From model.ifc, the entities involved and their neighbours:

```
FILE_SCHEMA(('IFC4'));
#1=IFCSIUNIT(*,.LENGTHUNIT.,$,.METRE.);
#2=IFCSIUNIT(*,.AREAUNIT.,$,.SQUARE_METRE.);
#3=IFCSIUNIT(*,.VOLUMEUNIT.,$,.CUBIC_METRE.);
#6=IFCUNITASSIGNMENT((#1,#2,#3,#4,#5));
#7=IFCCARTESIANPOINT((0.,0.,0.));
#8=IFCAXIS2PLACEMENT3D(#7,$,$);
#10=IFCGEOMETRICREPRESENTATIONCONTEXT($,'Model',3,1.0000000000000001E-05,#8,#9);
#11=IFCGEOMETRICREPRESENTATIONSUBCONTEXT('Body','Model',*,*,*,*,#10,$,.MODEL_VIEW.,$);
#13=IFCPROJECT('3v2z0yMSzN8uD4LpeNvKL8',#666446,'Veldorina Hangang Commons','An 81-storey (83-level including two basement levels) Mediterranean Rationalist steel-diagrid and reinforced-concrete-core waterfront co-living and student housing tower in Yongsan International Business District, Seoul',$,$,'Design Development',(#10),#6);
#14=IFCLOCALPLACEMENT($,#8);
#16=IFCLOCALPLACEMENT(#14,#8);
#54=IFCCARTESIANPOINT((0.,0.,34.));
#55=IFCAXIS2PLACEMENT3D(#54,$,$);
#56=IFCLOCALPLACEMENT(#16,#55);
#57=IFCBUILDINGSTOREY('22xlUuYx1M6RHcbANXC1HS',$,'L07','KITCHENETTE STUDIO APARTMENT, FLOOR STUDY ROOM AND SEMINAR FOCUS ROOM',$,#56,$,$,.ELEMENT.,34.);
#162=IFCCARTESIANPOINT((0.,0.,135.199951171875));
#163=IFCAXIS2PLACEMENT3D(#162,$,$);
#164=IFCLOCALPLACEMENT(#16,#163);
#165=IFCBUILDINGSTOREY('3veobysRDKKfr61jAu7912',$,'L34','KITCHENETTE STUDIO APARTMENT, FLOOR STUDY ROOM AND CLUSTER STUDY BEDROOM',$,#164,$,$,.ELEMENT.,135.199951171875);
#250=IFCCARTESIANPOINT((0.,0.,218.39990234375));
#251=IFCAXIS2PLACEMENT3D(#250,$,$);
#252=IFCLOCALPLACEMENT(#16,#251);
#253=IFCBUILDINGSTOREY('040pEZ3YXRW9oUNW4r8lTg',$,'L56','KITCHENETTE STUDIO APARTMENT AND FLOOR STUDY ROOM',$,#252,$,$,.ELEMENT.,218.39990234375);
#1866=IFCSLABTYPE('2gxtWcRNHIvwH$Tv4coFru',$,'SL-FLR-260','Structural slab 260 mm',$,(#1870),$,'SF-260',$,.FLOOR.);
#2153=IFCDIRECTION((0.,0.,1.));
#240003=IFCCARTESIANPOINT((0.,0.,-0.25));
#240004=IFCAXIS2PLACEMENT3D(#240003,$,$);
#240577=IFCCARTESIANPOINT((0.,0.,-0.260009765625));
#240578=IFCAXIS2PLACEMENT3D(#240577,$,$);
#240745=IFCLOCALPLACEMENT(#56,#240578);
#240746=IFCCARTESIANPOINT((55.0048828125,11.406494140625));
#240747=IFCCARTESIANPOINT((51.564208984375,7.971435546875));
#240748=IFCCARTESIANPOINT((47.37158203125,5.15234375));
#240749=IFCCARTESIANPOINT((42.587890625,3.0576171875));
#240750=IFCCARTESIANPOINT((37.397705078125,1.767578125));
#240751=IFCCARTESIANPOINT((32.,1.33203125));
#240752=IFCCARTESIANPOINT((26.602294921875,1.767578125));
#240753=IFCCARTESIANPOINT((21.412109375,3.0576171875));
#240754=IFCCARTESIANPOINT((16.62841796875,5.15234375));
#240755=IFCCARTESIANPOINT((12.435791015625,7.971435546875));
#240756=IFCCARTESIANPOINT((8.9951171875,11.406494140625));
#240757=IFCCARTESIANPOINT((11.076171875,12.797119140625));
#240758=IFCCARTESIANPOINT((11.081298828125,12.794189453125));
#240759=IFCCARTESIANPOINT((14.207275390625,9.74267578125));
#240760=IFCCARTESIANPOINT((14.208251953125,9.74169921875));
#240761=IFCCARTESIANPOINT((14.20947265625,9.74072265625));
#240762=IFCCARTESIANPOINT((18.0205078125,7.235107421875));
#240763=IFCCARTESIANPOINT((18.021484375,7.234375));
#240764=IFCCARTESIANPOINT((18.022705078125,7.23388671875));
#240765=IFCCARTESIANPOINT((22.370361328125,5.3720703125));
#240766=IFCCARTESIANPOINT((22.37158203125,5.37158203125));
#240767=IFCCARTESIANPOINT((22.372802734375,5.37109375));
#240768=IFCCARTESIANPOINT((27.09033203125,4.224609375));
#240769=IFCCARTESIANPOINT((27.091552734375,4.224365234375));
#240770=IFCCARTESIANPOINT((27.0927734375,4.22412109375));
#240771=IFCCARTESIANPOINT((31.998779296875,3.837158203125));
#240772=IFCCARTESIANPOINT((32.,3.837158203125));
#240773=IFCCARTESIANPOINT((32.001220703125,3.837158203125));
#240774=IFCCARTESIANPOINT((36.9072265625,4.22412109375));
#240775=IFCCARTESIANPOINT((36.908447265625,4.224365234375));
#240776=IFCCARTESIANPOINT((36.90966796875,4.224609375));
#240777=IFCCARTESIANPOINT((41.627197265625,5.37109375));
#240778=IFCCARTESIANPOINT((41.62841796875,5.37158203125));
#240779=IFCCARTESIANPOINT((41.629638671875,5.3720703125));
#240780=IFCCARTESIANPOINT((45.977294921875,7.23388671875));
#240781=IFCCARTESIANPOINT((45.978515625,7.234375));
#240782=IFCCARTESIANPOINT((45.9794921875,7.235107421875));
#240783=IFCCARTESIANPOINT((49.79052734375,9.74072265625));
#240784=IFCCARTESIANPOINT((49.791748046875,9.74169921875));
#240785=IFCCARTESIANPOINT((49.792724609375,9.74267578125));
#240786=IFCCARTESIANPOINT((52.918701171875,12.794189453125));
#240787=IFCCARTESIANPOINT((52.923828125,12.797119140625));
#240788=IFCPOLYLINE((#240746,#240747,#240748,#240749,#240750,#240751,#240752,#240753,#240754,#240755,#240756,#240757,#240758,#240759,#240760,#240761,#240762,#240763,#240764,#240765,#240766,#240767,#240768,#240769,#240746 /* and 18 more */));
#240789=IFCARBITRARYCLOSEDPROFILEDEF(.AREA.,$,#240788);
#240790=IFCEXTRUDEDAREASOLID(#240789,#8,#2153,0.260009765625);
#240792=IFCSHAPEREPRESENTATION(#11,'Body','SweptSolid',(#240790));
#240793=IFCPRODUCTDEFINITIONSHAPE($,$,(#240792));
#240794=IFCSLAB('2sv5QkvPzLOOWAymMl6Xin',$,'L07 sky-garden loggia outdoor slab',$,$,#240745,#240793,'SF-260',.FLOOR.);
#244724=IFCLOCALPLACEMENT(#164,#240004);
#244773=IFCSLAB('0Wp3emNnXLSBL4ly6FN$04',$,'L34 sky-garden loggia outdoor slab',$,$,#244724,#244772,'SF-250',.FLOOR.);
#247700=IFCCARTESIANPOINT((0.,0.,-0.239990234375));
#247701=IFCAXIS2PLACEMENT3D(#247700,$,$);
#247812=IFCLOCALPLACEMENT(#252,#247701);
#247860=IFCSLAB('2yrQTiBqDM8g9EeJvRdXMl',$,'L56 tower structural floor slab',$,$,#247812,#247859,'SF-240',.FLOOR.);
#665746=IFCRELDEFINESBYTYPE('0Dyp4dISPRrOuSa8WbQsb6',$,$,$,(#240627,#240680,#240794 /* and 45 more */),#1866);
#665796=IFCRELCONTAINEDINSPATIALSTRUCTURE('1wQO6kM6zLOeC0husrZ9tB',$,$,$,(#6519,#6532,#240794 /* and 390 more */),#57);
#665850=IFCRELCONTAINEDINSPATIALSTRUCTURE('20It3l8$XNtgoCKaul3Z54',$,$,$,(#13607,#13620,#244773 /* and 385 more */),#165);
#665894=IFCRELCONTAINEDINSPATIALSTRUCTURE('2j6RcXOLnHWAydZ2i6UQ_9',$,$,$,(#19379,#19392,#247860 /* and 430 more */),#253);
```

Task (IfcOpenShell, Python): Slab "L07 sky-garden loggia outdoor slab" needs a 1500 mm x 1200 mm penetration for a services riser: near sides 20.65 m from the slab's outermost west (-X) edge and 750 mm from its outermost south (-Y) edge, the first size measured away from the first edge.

```python
import numpy as np
import ifcopenshell
import ifcopenshell.api.feature
import ifcopenshell.api.geometry
import ifcopenshell.api.root
import ifcopenshell.geom
import ifcopenshell.util.placement
import ifcopenshell.util.representation
import ifcopenshell.util.shape
import ifcopenshell.util.unit

model = ifcopenshell.open("model.ifc")
unit_scale = ifcopenshell.util.unit.calculate_unit_scale(model)
settings = ifcopenshell.geom.settings()


def volume(element):
    """Net volume in cubic metres, openings subtracted."""
    shape = ifcopenshell.geom.create_shape(settings, element)
    return ifcopenshell.util.shape.get_volume(shape.geometry)


slab = model.by_guid("2sv5QkvPzLOOWAymMl6Xin")
before = volume(slab)

# Extent in the slab's own axes, in metres. The edges named are its -X and -Y sides.
slab_shape = ifcopenshell.geom.create_shape(settings, slab)
vertices = ifcopenshell.util.shape.get_vertices(slab_shape.geometry)
x_min, y_min, bottom = vertices.min(axis=0)
top = vertices[:, 2].max()

opening = ifcopenshell.api.root.create_entity(model, ifc_class="IfcOpeningElement", name="Services riser opening", predefined_type="OPENING")
context = ifcopenshell.util.representation.get_context(model, "Model", "Body", "MODEL_VIEW")
width, depth = 1.5, 1.2
outline = [(0.0, 0.0), (width, 0.0), (width, depth), (0.0, depth), (0.0, 0.0)]
# Overshoot both faces by 50 mm so the cut is clean.
shape = ifcopenshell.api.geometry.add_slab_representation(
    model, context=context, depth=top - bottom + 0.1, polyline=outline
)
ifcopenshell.api.geometry.assign_representation(model, product=opening, representation=shape)

matrix = ifcopenshell.util.placement.get_local_placement(slab.ObjectPlacement)
matrix[:, 3] = matrix @ np.append(np.array([x_min + 20.65, y_min + 0.75, bottom - 0.05]) / unit_scale, 1.0)
ifcopenshell.api.geometry.edit_object_placement(model, product=opening, matrix=matrix, is_si=False)
ifcopenshell.api.feature.add_feature(model, feature=opening, element=slab)

after = volume(slab)

print(f"slab volume {before:.3f} -> {after:.3f} m3")

model.write("model_rev.ifc")
```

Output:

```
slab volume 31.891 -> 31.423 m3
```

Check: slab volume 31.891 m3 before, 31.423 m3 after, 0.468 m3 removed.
